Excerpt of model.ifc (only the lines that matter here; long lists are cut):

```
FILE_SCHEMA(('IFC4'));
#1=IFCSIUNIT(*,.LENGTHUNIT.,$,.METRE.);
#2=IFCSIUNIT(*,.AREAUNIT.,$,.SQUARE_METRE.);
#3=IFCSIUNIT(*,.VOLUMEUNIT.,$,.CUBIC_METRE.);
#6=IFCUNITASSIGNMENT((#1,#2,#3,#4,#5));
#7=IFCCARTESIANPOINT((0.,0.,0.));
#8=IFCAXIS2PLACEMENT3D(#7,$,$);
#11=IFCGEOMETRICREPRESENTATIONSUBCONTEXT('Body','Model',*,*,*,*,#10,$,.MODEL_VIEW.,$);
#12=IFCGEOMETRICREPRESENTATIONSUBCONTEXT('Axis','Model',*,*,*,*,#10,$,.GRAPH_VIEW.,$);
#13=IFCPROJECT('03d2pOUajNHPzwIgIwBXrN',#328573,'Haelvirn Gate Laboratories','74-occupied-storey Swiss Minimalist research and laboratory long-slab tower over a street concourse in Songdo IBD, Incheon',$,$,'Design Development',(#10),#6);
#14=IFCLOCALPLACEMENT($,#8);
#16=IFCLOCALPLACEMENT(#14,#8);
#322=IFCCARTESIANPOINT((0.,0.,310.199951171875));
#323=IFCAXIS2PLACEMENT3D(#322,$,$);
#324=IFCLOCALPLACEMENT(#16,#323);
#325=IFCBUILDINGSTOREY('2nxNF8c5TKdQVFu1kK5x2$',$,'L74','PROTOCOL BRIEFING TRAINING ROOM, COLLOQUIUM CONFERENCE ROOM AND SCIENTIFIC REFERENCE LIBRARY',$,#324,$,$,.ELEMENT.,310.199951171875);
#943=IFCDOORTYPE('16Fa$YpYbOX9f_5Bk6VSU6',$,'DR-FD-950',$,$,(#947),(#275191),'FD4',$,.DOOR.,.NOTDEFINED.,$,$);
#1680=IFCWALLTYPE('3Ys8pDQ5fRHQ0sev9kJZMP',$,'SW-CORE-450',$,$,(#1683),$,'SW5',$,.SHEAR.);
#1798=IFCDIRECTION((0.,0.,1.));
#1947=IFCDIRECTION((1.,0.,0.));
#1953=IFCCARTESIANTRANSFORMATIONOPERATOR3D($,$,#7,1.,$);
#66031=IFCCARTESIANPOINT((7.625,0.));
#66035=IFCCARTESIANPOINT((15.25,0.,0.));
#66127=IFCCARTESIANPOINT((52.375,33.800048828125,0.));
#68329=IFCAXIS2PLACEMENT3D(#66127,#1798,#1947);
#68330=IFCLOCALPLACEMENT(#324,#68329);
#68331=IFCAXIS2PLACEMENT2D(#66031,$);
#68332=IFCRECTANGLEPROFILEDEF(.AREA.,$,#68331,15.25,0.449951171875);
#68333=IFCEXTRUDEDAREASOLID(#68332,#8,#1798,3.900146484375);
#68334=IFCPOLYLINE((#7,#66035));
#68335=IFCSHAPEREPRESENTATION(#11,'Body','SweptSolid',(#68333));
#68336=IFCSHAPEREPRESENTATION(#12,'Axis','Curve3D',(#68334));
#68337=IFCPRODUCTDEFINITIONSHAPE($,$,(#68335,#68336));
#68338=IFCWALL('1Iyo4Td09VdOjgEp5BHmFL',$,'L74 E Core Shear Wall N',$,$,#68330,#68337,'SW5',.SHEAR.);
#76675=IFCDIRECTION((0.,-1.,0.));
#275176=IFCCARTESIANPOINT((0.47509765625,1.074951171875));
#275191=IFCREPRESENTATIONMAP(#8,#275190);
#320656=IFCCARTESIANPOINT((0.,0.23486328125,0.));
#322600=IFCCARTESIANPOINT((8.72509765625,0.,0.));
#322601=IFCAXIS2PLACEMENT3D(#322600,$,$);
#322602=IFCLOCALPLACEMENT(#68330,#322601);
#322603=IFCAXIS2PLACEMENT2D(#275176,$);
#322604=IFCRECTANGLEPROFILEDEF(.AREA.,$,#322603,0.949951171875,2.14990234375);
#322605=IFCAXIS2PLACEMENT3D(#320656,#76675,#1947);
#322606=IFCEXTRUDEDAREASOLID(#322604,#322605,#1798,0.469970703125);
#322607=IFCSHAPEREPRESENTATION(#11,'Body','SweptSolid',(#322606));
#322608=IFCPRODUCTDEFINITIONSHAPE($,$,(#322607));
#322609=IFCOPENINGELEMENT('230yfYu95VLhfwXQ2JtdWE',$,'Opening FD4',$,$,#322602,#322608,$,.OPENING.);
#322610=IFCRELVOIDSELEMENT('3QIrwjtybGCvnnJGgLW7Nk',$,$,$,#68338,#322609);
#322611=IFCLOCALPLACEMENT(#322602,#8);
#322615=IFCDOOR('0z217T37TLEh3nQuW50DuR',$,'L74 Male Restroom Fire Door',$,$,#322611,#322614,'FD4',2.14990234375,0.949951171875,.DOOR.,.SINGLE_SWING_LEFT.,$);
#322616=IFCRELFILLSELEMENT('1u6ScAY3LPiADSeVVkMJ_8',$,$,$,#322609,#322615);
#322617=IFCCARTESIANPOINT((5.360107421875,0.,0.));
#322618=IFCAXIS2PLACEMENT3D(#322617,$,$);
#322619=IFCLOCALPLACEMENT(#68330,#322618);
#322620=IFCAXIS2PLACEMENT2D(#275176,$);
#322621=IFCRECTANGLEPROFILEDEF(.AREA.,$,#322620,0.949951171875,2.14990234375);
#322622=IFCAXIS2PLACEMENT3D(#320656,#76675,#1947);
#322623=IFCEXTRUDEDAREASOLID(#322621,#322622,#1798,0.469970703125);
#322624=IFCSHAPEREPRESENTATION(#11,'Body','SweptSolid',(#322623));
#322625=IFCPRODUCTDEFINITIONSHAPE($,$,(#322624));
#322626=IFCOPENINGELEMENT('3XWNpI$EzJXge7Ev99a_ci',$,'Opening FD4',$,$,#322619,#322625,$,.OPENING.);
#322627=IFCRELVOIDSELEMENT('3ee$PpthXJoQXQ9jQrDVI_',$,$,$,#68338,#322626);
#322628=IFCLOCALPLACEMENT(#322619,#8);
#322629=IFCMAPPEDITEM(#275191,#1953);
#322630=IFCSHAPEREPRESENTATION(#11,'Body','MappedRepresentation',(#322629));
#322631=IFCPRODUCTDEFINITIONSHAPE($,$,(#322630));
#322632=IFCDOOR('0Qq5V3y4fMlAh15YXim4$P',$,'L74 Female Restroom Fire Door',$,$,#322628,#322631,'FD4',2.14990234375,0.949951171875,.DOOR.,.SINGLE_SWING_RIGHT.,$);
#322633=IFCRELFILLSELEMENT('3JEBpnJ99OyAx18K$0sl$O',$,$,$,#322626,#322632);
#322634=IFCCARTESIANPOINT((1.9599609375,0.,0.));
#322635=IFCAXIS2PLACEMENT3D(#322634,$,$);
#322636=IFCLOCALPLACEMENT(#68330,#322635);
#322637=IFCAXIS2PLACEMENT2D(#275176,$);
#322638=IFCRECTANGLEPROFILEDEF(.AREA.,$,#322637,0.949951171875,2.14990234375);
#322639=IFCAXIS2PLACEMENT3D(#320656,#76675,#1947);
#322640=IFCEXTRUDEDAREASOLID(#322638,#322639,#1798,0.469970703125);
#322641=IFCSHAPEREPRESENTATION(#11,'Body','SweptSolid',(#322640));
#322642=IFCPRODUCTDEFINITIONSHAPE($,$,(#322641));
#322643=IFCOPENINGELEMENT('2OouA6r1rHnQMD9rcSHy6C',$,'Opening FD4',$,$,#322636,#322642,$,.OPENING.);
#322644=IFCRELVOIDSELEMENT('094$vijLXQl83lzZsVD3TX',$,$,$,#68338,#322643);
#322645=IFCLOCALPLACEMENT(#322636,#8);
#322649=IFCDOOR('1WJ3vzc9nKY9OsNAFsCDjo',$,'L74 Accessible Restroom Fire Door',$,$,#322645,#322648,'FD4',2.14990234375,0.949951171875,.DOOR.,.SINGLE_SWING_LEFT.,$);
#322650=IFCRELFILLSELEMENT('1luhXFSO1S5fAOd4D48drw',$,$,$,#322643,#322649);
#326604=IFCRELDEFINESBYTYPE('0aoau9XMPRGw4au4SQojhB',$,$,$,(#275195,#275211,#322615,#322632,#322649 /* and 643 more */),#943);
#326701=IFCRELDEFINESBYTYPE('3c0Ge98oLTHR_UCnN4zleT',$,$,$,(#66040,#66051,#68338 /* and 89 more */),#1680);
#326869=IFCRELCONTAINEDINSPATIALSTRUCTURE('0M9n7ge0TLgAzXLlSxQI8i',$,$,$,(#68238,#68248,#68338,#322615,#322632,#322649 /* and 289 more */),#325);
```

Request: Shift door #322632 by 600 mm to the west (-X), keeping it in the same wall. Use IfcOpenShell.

```python
import ifcopenshell
import ifcopenshell.api.geometry
import ifcopenshell.util.placement

model = ifcopenshell.open("model.ifc")

door = model.by_guid("0Qq5V3y4fMlAh15YXim4$P")
opening = door.FillsVoids[0].RelatingOpeningElement
wall = opening.VoidsElements[0].RelatingBuildingElement

wall_matrix = ifcopenshell.util.placement.get_local_placement(wall.ObjectPlacement)
shift = wall_matrix[:3, 0] * -0.6
before = ifcopenshell.util.placement.get_local_placement(door.ObjectPlacement)[:3, 3].copy()

# The door is placed relative to its opening, so it follows when the opening moves.
matrix = ifcopenshell.util.placement.get_local_placement(opening.ObjectPlacement)
matrix[:3, 3] += shift
ifcopenshell.api.geometry.edit_object_placement(
    model, product=opening, matrix=matrix, is_si=False, should_transform_children=True
)

after = ifcopenshell.util.placement.get_local_placement(door.ObjectPlacement)[:3, 3]
print("door moved by", (after - before).round(3) + 0.0)

model.write("model_updated.ifc")
```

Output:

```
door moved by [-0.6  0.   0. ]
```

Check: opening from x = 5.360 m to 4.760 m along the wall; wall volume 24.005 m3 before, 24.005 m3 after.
